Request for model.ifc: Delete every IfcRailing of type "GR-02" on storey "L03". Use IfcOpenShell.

First a look at what the model holds.

```python
import ifcopenshell
import ifcopenshell.util.element

model = ifcopenshell.open("model.ifc")
print(model.schema)
storey = next(s for s in model.by_type("IfcBuildingStorey") if s.Name == "L03")
railings = [e for e in ifcopenshell.util.element.get_decomposition(storey) if e.is_a("IfcRailing")]
seen = {}
for e in railings:
    element_type = ifcopenshell.util.element.get_type(e)
    name = element_type.Name if element_type not in (None, e) else None
    seen[name] = seen.get(name, 0) + 1
for name, count in sorted(seen.items(), key=str):
    print(count, "x", name)
```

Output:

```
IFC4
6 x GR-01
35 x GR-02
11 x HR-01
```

```python
import ifcopenshell
import ifcopenshell.api.root
import ifcopenshell.util.element

model = ifcopenshell.open("model.ifc")

storey = next(s for s in model.by_type("IfcBuildingStorey") if s.Name == "L03")
railings = [e for e in ifcopenshell.util.element.get_decomposition(storey) if e.is_a("IfcRailing")]
targets = [e for e in railings if (t := ifcopenshell.util.element.get_type(e)) not in (None, e) and t.Name == "GR-02"]

for e in targets:
    ifcopenshell.api.root.remove_product(model, product=e)
print(len(targets), "removed")

model.write("model_v2.ifc")
```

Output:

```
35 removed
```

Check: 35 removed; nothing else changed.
